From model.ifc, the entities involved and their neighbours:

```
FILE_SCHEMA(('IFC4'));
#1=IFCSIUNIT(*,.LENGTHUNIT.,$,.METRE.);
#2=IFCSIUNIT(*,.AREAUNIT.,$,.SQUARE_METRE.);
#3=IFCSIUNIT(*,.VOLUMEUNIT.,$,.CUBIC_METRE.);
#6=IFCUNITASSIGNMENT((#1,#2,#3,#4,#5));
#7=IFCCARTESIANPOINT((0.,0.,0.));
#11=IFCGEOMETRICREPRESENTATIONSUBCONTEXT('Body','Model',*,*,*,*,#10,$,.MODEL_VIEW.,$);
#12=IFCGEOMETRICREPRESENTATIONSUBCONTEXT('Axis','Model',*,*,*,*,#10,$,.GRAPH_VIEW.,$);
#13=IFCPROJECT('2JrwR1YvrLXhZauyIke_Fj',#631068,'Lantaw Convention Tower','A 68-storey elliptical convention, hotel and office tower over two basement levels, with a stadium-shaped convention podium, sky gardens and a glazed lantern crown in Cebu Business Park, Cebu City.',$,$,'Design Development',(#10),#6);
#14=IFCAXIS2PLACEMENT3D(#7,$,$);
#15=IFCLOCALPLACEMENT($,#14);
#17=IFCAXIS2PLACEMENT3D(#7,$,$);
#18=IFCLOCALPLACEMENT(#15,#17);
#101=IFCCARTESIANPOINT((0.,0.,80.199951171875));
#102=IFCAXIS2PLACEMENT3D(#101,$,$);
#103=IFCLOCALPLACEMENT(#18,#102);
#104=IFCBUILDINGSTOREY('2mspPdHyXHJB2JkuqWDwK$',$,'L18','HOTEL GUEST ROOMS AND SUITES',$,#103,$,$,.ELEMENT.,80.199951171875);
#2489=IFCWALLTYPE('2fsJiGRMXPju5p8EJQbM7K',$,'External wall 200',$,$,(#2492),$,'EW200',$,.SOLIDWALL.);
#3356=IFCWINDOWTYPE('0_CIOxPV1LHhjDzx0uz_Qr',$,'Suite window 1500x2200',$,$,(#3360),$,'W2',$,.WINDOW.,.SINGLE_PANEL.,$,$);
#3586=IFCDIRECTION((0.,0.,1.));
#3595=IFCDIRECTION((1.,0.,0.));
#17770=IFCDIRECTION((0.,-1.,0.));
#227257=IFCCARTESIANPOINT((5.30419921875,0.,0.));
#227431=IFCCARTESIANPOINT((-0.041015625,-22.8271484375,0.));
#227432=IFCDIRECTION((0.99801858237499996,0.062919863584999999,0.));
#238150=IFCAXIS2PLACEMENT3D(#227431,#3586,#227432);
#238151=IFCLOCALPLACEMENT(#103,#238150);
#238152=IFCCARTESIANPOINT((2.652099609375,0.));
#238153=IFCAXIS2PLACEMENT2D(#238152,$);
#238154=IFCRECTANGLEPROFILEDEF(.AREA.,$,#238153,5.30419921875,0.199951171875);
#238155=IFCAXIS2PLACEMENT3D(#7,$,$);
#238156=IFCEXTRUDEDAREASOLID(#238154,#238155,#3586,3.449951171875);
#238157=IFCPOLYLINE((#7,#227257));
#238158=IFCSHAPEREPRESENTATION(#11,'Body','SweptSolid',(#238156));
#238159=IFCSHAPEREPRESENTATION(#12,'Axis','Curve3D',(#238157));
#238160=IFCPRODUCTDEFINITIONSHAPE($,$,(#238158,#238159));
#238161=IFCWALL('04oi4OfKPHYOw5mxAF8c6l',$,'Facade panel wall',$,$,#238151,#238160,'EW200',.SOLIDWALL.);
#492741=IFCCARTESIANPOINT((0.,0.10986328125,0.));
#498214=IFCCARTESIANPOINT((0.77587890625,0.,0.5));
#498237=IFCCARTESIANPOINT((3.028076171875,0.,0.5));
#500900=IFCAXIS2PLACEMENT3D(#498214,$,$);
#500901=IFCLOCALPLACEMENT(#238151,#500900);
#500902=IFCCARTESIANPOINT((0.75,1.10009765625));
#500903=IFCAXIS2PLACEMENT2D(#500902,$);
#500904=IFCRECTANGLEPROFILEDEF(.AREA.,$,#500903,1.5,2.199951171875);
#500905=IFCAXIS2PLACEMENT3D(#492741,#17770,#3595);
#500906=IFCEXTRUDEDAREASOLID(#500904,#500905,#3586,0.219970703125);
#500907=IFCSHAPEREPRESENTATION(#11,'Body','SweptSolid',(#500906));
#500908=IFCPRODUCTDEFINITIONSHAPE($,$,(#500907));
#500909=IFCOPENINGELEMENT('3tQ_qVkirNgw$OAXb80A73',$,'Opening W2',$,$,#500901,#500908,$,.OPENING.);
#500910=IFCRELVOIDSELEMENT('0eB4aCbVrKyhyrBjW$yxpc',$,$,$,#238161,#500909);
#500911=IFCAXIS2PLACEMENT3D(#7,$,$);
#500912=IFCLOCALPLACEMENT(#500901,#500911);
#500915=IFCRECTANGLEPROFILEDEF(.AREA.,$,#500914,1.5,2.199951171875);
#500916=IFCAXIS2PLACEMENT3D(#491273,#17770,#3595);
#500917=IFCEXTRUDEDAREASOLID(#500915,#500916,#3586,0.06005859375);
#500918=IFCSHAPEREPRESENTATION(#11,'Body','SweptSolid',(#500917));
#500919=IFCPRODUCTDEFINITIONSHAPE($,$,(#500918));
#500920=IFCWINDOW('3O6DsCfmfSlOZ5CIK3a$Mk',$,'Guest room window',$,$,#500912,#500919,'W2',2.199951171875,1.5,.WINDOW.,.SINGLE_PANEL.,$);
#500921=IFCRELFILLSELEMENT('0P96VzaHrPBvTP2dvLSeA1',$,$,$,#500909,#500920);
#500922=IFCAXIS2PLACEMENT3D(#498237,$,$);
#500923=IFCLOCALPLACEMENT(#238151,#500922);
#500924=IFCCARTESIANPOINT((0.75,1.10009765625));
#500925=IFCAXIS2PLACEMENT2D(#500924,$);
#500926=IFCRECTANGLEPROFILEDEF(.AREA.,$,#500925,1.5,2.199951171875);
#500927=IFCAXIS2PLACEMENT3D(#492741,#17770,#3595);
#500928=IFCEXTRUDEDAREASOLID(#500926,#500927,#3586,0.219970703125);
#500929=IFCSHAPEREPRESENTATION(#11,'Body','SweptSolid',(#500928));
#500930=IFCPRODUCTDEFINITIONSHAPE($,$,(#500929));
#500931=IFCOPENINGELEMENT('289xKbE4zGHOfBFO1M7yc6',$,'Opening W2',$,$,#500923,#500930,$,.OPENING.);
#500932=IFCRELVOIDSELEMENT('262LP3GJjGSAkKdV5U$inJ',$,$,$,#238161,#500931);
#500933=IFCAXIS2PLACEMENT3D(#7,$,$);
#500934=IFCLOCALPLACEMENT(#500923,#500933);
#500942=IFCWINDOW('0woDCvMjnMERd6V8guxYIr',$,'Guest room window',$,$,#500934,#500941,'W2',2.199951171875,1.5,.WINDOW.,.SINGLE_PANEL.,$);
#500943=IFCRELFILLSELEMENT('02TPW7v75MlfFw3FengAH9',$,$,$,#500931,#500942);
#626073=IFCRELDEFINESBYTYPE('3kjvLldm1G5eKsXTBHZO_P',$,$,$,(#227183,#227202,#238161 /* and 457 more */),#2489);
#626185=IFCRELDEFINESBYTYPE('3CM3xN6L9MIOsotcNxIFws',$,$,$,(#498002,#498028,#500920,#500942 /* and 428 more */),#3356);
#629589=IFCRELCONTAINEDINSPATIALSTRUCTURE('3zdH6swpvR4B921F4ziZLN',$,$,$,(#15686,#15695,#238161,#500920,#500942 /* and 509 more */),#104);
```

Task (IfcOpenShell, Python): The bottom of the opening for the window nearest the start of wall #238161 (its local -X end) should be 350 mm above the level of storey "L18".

```python
import numpy as np
import ifcopenshell
import ifcopenshell.api.geometry
import ifcopenshell.geom
import ifcopenshell.util.element
import ifcopenshell.util.placement
import ifcopenshell.util.shape
import ifcopenshell.util.unit

model = ifcopenshell.open("model.ifc")
unit_scale = ifcopenshell.util.unit.calculate_unit_scale(model)

window = model.by_id(500920)
opening = window.FillsVoids[0].RelatingOpeningElement
storey = ifcopenshell.util.element.get_container(window, ifc_class="IfcBuildingStorey")
level = ifcopenshell.util.placement.get_local_placement(storey.ObjectPlacement)[2, 3]

# The opening's origin need not be at the sill, so measure its lowest point.
shape = ifcopenshell.geom.create_shape(ifcopenshell.geom.settings(), opening)
bottom = ifcopenshell.util.shape.get_shape_bottom_elevation(shape, shape.geometry) / unit_scale
dz = level + 0.35 - bottom

shift = np.array([0.0, 0.0, dz])
# The window is placed relative to its opening, so it follows when the opening moves.
matrix = ifcopenshell.util.placement.get_local_placement(opening.ObjectPlacement)
matrix[:3, 3] += shift
ifcopenshell.api.geometry.edit_object_placement(
    model, product=opening, matrix=matrix, is_si=False, should_transform_children=True
)

print(f"moved by {dz * unit_scale:+.3f} m")

model.write("model_rev.ifc")
```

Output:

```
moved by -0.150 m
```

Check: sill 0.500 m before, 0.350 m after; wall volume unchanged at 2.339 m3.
